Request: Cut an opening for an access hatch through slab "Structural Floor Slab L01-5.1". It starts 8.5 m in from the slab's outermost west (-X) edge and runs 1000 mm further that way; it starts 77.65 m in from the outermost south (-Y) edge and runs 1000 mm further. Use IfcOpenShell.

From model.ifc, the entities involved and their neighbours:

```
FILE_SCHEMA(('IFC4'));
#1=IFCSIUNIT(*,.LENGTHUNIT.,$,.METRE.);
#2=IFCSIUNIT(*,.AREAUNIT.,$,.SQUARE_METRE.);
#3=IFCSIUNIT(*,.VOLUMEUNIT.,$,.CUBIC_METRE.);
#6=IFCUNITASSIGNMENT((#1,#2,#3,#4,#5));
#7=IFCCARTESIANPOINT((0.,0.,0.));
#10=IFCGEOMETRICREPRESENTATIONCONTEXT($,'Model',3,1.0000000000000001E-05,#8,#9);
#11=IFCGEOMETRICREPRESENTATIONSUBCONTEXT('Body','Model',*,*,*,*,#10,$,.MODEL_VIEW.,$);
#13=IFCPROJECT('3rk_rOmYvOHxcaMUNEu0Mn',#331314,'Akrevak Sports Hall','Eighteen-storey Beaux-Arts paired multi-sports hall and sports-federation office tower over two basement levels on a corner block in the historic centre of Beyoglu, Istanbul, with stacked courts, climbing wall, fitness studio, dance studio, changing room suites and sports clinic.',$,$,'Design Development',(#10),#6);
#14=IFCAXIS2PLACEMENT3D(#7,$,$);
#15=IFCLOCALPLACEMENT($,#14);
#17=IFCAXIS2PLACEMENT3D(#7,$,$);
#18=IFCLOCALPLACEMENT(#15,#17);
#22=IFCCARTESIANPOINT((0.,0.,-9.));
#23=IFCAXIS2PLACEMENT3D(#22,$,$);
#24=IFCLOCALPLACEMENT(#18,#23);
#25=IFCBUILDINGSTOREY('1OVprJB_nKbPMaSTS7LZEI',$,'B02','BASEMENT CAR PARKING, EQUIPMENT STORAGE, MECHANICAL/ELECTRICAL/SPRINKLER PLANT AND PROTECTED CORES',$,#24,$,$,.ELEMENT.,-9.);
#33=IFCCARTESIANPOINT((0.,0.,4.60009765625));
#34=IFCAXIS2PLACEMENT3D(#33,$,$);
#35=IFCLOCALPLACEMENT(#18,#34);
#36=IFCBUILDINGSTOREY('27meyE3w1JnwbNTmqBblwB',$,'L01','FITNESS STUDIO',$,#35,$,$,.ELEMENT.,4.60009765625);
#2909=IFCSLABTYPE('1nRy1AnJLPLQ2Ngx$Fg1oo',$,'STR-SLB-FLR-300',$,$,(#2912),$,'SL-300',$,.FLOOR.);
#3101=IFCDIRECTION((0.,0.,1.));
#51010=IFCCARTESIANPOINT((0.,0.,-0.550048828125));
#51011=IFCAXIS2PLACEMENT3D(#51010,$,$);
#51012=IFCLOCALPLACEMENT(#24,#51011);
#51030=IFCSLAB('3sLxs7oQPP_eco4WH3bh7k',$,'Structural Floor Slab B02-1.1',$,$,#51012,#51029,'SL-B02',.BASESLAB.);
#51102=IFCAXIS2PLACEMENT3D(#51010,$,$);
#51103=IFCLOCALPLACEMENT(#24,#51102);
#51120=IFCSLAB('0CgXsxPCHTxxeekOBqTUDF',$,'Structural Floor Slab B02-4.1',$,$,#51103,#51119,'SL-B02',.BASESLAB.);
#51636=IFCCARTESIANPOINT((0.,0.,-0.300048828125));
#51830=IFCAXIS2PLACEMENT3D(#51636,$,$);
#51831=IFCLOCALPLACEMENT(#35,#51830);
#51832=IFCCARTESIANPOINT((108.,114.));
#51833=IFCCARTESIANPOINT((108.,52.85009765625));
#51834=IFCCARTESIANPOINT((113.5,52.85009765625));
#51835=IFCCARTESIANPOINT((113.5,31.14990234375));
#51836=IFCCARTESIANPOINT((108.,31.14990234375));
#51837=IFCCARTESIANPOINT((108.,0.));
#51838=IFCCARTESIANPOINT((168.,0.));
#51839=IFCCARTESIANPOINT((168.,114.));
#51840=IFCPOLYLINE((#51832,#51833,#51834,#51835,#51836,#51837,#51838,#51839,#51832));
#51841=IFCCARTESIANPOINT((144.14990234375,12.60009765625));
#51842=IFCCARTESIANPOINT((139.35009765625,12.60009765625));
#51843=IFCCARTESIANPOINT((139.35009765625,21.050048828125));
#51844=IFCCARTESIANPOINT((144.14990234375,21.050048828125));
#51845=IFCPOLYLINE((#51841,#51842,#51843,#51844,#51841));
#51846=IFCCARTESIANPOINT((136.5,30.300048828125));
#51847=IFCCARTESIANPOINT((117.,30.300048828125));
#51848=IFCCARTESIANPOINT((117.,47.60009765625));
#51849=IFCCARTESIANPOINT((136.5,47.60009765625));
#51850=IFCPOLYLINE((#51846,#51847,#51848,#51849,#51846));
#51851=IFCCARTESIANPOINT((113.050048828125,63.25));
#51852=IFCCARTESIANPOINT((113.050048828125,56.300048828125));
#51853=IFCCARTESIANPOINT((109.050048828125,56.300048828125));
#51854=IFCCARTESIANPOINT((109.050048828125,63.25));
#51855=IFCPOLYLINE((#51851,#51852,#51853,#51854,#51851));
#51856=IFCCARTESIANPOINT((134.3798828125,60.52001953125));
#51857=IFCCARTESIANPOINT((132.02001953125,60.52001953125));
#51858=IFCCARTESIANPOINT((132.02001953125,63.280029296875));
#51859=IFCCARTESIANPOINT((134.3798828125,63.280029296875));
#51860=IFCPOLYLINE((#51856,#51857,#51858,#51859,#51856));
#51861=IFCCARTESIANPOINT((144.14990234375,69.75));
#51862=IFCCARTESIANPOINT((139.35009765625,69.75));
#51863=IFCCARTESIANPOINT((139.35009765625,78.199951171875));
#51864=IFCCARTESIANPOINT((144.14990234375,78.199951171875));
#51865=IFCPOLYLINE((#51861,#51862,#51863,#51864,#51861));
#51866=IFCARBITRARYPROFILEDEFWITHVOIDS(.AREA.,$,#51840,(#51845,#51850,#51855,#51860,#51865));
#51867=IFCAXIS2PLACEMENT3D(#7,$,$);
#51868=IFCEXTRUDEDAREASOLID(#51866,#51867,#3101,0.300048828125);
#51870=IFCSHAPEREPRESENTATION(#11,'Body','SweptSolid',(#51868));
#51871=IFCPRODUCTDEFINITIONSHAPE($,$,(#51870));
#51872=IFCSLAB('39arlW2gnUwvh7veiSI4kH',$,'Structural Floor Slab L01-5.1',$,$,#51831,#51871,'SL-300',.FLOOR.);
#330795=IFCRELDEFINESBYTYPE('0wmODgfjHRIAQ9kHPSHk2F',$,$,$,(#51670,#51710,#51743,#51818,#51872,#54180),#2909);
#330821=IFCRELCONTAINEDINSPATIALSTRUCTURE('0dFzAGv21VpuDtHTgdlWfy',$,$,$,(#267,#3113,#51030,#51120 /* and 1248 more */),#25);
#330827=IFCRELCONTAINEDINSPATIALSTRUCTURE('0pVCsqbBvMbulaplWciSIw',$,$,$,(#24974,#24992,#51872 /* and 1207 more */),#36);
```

```python
import numpy as np
import ifcopenshell
import ifcopenshell.api.feature
import ifcopenshell.api.geometry
import ifcopenshell.api.root
import ifcopenshell.geom
import ifcopenshell.util.placement
import ifcopenshell.util.representation
import ifcopenshell.util.shape
import ifcopenshell.util.unit

model = ifcopenshell.open("model.ifc")
unit_scale = ifcopenshell.util.unit.calculate_unit_scale(model)
settings = ifcopenshell.geom.settings()


def volume(element):
    """Net volume in cubic metres, openings subtracted."""
    shape = ifcopenshell.geom.create_shape(settings, element)
    return ifcopenshell.util.shape.get_volume(shape.geometry)


slab = model.by_id(51872)
before = volume(slab)

# Extent in the slab's own axes, in metres. The edges named are its -X and -Y sides.
slab_shape = ifcopenshell.geom.create_shape(settings, slab)
vertices = ifcopenshell.util.shape.get_vertices(slab_shape.geometry)
x_min, y_min, bottom = vertices.min(axis=0)
top = vertices[:, 2].max()

opening = ifcopenshell.api.root.create_entity(model, ifc_class="IfcOpeningElement", name="Access hatch opening", predefined_type="OPENING")
context = ifcopenshell.util.representation.get_context(model, "Model", "Body", "MODEL_VIEW")
width, depth = 1, 1
outline = [(0.0, 0.0), (width, 0.0), (width, depth), (0.0, depth), (0.0, 0.0)]
# Overshoot both faces by 50 mm so the cut is clean.
shape = ifcopenshell.api.geometry.add_slab_representation(
    model, context=context, depth=top - bottom + 0.1, polyline=outline
)
ifcopenshell.api.geometry.assign_representation(model, product=opening, representation=shape)

matrix = ifcopenshell.util.placement.get_local_placement(slab.ObjectPlacement)
matrix[:, 3] = matrix @ np.append(np.array([x_min + 8.5, y_min + 77.65, bottom - 0.05]) / unit_scale, 1.0)
ifcopenshell.api.geometry.edit_object_placement(model, product=opening, matrix=matrix, is_si=False)
ifcopenshell.api.feature.add_feature(model, feature=opening, element=slab)

after = volume(slab)

print(f"slab volume {before:.3f} -> {after:.3f} m3")

model.write("model_v2.ifc")
```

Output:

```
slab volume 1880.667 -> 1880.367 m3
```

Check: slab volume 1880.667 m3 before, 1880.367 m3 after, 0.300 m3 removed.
